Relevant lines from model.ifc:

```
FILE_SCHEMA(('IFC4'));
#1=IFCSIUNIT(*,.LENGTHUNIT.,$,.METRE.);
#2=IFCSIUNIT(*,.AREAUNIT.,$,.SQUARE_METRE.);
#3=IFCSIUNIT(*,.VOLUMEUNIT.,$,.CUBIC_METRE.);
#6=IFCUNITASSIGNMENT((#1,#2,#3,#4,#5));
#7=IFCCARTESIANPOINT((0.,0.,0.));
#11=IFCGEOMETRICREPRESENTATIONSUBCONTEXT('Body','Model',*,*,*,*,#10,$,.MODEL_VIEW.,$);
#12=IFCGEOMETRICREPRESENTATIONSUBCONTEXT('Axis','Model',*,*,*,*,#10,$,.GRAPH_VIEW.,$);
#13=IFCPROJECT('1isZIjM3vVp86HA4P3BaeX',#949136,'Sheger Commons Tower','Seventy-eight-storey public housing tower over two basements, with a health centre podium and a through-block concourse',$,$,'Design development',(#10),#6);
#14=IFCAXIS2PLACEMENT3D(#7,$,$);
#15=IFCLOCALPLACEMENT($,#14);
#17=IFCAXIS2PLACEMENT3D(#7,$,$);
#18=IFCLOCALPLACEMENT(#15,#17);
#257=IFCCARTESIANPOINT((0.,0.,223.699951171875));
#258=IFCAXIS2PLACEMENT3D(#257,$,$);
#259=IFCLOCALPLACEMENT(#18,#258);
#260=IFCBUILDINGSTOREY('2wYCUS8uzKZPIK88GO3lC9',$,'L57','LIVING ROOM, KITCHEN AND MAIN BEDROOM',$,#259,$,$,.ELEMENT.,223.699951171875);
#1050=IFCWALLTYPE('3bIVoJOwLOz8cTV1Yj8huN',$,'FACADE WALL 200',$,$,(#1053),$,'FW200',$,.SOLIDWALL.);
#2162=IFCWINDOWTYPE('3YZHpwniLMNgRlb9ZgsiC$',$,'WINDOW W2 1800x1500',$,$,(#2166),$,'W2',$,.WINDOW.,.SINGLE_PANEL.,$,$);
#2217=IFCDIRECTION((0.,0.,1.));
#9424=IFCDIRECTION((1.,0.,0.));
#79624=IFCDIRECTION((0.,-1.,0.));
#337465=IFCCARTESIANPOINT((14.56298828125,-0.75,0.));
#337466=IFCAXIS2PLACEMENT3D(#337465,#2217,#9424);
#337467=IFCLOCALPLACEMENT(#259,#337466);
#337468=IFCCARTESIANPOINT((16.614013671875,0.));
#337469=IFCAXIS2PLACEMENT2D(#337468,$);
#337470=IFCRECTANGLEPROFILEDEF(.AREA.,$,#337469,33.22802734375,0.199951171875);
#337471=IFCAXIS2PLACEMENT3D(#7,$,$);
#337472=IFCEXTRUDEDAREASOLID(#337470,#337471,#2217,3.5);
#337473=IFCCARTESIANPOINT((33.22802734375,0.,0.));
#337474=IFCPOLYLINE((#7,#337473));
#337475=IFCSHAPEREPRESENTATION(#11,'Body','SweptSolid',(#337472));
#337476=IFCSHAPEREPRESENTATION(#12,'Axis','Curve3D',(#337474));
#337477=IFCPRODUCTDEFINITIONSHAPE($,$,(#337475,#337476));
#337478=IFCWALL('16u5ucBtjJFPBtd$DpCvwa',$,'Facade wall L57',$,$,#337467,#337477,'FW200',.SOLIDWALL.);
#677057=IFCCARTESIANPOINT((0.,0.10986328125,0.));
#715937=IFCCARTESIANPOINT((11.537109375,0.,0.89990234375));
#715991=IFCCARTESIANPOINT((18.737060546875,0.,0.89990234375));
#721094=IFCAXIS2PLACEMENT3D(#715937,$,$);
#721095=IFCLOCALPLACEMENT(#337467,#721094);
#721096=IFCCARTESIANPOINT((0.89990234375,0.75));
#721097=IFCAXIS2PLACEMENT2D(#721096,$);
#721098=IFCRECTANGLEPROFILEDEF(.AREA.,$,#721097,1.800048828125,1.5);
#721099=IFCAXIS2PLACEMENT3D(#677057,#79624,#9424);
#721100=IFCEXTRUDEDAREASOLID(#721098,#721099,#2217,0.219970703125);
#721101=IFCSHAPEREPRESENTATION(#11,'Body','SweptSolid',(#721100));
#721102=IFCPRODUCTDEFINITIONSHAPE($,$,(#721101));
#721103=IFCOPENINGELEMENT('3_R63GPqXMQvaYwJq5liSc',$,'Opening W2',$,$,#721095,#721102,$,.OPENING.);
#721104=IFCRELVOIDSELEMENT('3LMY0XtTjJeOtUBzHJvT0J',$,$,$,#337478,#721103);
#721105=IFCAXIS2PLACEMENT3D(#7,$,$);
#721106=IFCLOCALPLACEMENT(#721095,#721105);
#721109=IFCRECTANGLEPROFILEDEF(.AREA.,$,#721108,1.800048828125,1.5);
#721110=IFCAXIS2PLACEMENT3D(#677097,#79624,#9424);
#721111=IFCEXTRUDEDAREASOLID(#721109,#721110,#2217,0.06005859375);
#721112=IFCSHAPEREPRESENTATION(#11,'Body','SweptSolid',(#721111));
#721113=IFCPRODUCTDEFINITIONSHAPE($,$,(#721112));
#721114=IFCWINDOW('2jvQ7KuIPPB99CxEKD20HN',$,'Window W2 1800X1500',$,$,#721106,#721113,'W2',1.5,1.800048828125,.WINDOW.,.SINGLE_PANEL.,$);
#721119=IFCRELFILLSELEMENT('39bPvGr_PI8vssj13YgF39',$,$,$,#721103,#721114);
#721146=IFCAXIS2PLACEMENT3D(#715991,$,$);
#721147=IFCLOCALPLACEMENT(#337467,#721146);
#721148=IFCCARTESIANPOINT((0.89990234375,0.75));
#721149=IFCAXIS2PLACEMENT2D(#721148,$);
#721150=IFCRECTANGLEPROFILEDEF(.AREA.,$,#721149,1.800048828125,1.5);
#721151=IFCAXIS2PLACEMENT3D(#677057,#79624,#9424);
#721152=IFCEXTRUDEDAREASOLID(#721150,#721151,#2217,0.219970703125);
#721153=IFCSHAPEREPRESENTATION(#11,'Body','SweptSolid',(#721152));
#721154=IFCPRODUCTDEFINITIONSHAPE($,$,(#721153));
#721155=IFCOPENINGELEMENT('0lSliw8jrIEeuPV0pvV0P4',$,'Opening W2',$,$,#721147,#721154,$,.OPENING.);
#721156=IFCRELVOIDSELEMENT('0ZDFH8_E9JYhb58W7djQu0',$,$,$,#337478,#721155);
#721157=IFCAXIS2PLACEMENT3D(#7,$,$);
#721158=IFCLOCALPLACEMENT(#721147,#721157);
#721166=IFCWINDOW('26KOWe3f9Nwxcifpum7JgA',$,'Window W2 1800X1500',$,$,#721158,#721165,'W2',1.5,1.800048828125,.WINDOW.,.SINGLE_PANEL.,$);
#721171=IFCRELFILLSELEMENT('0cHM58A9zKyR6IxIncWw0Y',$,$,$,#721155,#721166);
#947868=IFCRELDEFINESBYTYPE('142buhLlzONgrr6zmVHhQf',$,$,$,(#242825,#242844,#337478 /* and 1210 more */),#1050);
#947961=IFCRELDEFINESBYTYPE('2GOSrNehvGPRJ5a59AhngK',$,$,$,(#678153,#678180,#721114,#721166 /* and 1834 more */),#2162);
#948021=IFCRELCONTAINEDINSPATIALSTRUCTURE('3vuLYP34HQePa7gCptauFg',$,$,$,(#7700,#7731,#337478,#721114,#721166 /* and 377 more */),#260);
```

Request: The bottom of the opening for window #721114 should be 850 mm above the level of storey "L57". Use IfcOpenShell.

```python
import numpy as np
import ifcopenshell
import ifcopenshell.api.geometry
import ifcopenshell.geom
import ifcopenshell.util.element
import ifcopenshell.util.placement
import ifcopenshell.util.shape
import ifcopenshell.util.unit

model = ifcopenshell.open("model.ifc")
unit_scale = ifcopenshell.util.unit.calculate_unit_scale(model)

window = model.by_guid("2jvQ7KuIPPB99CxEKD20HN")
opening = window.FillsVoids[0].RelatingOpeningElement
storey = ifcopenshell.util.element.get_container(window, ifc_class="IfcBuildingStorey")
level = ifcopenshell.util.placement.get_local_placement(storey.ObjectPlacement)[2, 3]

# The opening's origin need not be at the sill, so measure its lowest point.
shape = ifcopenshell.geom.create_shape(ifcopenshell.geom.settings(), opening)
bottom = ifcopenshell.util.shape.get_shape_bottom_elevation(shape, shape.geometry) / unit_scale
dz = level + 0.85 / unit_scale - bottom

shift = np.array([0.0, 0.0, dz])
# The window is placed relative to its opening, so it follows when the opening moves.
matrix = ifcopenshell.util.placement.get_local_placement(opening.ObjectPlacement)
matrix[:3, 3] += shift
ifcopenshell.api.geometry.edit_object_placement(
    model, product=opening, matrix=matrix, is_si=False, should_transform_children=True
)

print(f"moved by {dz * unit_scale:+.3f} m")

model.write("model_rev.ifc")
```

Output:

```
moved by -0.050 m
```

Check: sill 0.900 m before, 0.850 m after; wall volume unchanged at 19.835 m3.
